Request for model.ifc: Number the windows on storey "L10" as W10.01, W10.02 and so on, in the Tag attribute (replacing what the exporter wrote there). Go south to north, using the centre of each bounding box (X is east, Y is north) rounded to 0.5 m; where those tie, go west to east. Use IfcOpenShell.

First a look at what the model holds.

```python
import ifcopenshell
import ifcopenshell.util.element
import ifcopenshell.util.placement

model = ifcopenshell.open("model.ifc")
print(model.schema)
storey = next(s for s in model.by_type("IfcBuildingStorey") if s.Name == "L10")
windows = [e for e in ifcopenshell.util.element.get_decomposition(storey) if e.is_a("IfcWindow")]
for e in sorted(windows, key=lambda e: e.id()):
    origin = ifcopenshell.util.placement.get_local_placement(e.ObjectPlacement)[:3, 3]
    print(e.id(), e.Tag, e.Name, origin.round(2) + 0.0, sep=" | ")
```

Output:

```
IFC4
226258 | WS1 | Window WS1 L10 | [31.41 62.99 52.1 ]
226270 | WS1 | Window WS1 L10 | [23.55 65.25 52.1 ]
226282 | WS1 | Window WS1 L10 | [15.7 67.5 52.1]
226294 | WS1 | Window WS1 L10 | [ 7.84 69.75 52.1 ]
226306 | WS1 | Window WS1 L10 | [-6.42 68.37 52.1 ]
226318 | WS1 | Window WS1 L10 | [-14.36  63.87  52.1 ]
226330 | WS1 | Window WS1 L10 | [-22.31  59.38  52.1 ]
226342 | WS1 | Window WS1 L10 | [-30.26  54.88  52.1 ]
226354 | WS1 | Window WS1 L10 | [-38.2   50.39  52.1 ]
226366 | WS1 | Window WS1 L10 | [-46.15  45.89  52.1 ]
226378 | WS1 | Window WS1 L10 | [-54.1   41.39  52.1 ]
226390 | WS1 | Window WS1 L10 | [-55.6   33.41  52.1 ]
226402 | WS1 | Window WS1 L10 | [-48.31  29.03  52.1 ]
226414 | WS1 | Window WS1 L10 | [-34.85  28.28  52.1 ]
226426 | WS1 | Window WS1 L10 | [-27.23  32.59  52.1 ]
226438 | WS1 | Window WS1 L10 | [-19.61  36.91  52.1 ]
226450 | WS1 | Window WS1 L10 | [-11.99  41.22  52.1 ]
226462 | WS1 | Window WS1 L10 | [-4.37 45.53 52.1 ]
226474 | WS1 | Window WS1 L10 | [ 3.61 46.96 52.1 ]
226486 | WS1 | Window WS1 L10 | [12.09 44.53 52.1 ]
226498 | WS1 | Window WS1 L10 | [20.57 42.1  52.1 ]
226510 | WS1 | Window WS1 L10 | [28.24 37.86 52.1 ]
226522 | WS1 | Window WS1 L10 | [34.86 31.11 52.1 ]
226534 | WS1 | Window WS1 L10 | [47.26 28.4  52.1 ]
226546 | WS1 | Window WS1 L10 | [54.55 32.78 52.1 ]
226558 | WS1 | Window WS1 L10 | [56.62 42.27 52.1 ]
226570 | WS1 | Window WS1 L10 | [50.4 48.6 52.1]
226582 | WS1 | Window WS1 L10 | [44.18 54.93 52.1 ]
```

```python
import ifcopenshell
import ifcopenshell.geom
import ifcopenshell.util.element
import ifcopenshell.util.shape

model = ifcopenshell.open("model.ifc")
settings = ifcopenshell.geom.settings()
settings.set("use-world-coords", True)


def centre(element):
    shape = ifcopenshell.geom.create_shape(settings, element)
    return ifcopenshell.util.shape.get_bbox_centroid(shape.geometry)


storey = next(s for s in model.by_type("IfcBuildingStorey") if s.Name == "L10")
windows = [e for e in ifcopenshell.util.element.get_decomposition(storey) if e.is_a("IfcWindow")]

# Insertion points can sit at a corner or the storey origin, so sort by the geometry (in metres).
centres = {e: centre(e) for e in windows}
windows.sort(key=lambda e: (round(centres[e][1] / 0.5), centres[e][0]))

for i, e in enumerate(windows, start=1):
    number = f"W10.{i:02d}"
    e.Tag = number
    print(e.id(), number)

model.write("model_edited.ifc")
```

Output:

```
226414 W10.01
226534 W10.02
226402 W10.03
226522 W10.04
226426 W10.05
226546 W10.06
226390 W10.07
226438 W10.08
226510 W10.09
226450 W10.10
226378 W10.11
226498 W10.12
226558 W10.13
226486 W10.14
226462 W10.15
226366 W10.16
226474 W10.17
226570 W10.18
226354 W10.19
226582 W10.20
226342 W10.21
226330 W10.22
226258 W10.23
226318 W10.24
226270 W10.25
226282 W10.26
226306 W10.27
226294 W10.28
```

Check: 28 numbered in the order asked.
